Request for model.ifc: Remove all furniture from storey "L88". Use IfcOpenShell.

First a look at what the model holds.

```python
import ifcopenshell
import ifcopenshell.util.element

model = ifcopenshell.open("model.ifc")
print(model.schema)
storey = next(s for s in model.by_type("IfcBuildingStorey") if s.Name == "L88")
furniture = [e for e in ifcopenshell.util.element.get_decomposition(storey) if e.is_a("IfcFurnishingElement")]
seen = {}
for e in furniture:
    element_type = ifcopenshell.util.element.get_type(e)
    name = element_type.Name if element_type not in (None, e) else None
    seen[name] = seen.get(name, 0) + 1
for name, count in sorted(seen.items(), key=str):
    print(count, "x", name)
```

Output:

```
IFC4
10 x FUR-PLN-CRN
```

```python
import ifcopenshell
import ifcopenshell.api.root
import ifcopenshell.util.element

model = ifcopenshell.open("model.ifc")

storey = next(s for s in model.by_type("IfcBuildingStorey") if s.Name == "L88")
furniture = [e for e in ifcopenshell.util.element.get_decomposition(storey) if e.is_a("IfcFurnishingElement")]

for e in furniture:
    ifcopenshell.api.root.remove_product(model, product=e)
print(len(furniture), "removed")

model.write("model_updated.ifc")
```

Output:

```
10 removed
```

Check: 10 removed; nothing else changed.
